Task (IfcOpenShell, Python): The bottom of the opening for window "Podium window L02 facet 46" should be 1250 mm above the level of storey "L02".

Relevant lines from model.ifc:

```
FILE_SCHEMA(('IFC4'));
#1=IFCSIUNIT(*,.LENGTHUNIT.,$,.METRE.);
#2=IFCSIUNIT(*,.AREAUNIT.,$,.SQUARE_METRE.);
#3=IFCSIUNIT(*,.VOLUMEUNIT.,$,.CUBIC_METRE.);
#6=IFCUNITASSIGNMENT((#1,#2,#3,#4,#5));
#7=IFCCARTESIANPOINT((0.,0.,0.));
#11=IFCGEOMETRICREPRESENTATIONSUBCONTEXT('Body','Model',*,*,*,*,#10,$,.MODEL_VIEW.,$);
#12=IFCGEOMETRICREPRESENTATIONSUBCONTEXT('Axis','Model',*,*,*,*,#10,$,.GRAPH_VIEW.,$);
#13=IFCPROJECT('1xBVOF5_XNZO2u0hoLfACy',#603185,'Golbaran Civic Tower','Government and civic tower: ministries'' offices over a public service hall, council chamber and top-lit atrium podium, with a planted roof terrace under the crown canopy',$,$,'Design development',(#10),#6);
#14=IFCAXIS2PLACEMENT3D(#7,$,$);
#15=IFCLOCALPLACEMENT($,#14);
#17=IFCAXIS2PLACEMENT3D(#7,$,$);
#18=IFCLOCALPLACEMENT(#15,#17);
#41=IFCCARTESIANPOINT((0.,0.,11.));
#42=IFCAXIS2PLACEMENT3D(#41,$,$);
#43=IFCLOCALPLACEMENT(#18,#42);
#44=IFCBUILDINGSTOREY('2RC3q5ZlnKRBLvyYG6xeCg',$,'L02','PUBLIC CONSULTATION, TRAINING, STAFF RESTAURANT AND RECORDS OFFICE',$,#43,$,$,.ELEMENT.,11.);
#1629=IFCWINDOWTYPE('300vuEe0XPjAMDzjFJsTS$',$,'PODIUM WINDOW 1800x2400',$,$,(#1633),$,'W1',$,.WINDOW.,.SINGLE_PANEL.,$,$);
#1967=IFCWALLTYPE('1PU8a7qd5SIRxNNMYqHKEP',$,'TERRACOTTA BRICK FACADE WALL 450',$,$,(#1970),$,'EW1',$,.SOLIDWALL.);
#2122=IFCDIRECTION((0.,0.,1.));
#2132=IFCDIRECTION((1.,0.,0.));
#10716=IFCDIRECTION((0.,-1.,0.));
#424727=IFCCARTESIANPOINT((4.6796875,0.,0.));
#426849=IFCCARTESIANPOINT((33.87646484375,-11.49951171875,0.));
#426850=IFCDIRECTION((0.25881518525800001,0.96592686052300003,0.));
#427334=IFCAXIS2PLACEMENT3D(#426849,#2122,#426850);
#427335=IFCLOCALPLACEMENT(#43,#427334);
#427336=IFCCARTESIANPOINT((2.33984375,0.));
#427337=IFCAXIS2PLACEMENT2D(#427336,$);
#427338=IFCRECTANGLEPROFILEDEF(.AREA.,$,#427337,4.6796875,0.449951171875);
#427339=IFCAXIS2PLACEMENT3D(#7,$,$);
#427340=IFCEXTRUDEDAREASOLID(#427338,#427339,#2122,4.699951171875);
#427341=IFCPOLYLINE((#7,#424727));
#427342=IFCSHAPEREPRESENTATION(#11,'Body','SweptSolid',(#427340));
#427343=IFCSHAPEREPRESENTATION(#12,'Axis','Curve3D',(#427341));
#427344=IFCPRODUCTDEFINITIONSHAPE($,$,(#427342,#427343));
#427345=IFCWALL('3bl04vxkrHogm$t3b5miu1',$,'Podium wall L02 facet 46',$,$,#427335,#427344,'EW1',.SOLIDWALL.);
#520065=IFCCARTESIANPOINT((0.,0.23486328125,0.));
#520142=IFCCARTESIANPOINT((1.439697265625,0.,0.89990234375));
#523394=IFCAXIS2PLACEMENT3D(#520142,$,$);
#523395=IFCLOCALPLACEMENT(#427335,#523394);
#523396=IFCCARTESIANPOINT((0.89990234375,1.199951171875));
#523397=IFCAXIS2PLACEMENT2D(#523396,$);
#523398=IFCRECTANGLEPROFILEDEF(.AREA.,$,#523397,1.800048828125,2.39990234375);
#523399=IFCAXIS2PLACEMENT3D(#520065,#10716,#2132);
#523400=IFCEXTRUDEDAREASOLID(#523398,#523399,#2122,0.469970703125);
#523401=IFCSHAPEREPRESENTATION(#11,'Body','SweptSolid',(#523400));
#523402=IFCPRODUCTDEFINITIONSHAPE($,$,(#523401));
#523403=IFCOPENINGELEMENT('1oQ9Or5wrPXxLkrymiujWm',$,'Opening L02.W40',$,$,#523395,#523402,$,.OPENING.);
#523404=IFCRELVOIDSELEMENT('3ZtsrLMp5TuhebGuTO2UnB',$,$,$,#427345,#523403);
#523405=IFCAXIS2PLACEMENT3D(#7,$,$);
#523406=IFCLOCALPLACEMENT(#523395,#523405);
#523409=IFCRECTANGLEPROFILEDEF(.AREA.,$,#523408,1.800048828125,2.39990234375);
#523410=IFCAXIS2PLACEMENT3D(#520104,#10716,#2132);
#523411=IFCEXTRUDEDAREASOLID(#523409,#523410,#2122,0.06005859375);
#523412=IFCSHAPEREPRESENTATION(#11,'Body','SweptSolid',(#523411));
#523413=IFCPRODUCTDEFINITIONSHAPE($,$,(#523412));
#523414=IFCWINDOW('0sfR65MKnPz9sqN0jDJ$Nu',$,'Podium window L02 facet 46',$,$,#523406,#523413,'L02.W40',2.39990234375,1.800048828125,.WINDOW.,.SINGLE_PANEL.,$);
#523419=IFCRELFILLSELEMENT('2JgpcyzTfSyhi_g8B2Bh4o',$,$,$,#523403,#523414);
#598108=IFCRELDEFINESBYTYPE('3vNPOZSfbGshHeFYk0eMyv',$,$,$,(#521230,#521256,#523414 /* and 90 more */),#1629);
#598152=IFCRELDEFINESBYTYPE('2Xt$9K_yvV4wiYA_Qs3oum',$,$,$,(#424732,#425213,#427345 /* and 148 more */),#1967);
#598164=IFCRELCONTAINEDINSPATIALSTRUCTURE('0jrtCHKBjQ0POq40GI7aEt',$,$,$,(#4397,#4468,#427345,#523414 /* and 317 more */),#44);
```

```python
import numpy as np
import ifcopenshell
import ifcopenshell.api.geometry
import ifcopenshell.geom
import ifcopenshell.util.element
import ifcopenshell.util.placement
import ifcopenshell.util.shape
import ifcopenshell.util.unit

model = ifcopenshell.open("model.ifc")
unit_scale = ifcopenshell.util.unit.calculate_unit_scale(model)

window = model.by_id(523414)
opening = window.FillsVoids[0].RelatingOpeningElement
storey = ifcopenshell.util.element.get_container(window, ifc_class="IfcBuildingStorey")
level = ifcopenshell.util.placement.get_local_placement(storey.ObjectPlacement)[2, 3]

# The opening's origin need not be at the sill, so measure its lowest point.
shape = ifcopenshell.geom.create_shape(ifcopenshell.geom.settings(), opening)
bottom = ifcopenshell.util.shape.get_shape_bottom_elevation(shape, shape.geometry) / unit_scale
dz = level + 1.25 / unit_scale - bottom

shift = np.array([0.0, 0.0, dz])
# The window is placed relative to its opening, so it follows when the opening moves.
matrix = ifcopenshell.util.placement.get_local_placement(opening.ObjectPlacement)
matrix[:3, 3] += shift
ifcopenshell.api.geometry.edit_object_placement(
    model, product=opening, matrix=matrix, is_si=False, should_transform_children=True
)

print(f"moved by {dz * unit_scale:+.3f} m")

model.write("model_updated.ifc")
```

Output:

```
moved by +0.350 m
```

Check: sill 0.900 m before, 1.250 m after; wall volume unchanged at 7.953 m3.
